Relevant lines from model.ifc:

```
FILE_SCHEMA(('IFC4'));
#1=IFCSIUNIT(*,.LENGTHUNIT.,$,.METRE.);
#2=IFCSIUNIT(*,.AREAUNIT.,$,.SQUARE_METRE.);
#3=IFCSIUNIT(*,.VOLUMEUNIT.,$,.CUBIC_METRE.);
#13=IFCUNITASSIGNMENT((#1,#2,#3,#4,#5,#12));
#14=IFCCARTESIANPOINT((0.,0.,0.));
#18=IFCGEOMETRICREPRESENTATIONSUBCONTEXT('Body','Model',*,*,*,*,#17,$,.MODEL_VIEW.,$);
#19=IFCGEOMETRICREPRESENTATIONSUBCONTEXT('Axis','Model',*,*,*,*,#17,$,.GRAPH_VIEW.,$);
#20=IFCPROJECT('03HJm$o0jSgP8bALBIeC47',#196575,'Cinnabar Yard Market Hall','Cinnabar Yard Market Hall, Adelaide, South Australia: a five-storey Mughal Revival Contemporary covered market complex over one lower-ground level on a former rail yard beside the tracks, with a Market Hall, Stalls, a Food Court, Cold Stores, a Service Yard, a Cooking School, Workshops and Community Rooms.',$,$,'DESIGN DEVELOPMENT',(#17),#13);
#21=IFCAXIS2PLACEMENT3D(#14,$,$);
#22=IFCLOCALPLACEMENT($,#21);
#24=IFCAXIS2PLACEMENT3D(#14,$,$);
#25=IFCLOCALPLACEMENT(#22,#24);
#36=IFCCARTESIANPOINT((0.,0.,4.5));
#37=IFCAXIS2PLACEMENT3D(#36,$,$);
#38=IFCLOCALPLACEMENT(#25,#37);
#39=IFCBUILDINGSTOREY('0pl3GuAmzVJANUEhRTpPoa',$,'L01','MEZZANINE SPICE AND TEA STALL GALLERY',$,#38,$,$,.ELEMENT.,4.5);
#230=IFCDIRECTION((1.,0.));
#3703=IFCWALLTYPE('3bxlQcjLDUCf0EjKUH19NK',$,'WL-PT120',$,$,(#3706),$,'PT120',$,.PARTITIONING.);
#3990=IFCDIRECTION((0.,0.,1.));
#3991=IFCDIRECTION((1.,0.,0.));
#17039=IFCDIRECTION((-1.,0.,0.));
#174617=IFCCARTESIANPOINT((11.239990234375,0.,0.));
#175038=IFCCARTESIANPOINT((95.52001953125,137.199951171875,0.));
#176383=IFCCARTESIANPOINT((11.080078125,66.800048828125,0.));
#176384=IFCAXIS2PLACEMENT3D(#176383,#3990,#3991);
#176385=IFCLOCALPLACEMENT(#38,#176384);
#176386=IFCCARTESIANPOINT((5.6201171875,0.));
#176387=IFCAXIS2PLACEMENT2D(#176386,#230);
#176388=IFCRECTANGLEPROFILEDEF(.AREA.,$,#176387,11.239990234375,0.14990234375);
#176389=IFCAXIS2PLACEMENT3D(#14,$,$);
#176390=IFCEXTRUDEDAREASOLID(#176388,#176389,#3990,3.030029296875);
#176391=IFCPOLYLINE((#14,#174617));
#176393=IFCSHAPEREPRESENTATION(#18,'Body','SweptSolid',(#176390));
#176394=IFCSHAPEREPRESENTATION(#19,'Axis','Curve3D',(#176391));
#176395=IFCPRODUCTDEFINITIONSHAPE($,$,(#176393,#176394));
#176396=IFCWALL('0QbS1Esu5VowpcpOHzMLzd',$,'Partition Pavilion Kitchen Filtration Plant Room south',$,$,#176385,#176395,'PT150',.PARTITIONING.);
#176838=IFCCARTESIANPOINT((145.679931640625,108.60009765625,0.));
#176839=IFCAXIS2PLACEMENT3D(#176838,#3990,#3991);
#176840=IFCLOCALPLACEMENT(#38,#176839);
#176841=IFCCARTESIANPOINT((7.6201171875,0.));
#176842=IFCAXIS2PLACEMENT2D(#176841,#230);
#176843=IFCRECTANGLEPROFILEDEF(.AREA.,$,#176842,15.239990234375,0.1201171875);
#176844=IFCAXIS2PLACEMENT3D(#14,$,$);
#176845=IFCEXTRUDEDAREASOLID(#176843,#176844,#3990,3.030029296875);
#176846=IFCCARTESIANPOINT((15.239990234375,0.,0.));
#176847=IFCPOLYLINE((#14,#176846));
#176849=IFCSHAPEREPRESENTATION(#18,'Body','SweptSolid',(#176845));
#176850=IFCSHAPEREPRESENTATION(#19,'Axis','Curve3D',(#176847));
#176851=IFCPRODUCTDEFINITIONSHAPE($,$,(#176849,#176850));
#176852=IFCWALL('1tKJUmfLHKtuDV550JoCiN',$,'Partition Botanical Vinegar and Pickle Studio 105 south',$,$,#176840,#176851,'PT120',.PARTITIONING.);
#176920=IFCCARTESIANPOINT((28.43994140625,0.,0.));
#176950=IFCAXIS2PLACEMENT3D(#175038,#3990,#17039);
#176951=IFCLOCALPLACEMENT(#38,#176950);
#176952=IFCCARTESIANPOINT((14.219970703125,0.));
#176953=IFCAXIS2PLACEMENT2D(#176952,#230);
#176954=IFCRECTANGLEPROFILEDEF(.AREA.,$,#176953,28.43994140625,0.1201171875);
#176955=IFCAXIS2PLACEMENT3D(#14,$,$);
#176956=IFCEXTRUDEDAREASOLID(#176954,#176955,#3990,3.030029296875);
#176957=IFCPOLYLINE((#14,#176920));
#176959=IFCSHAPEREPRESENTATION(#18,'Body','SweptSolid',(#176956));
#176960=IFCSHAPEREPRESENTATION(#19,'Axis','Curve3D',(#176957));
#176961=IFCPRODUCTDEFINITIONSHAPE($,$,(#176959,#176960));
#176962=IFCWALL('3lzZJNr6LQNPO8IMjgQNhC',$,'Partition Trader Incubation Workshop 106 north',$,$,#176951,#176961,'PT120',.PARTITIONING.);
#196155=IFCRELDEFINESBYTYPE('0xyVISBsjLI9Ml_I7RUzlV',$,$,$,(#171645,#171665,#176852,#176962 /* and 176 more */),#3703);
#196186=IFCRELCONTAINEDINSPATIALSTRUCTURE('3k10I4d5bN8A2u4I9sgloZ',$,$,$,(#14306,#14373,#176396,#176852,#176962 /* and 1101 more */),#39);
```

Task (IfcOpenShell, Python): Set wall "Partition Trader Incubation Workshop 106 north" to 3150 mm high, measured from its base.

```python
import ifcopenshell
import ifcopenshell.geom
import ifcopenshell.util.representation
import ifcopenshell.util.shape
import ifcopenshell.util.unit

model = ifcopenshell.open("model.ifc")
unit_scale = ifcopenshell.util.unit.calculate_unit_scale(model)
settings = ifcopenshell.geom.settings()


def volume(element):
    """Net volume in cubic metres, openings subtracted."""
    shape = ifcopenshell.geom.create_shape(settings, element)
    return ifcopenshell.util.shape.get_volume(shape.geometry)


wall = model.by_id(176962)
before = volume(wall)

body = ifcopenshell.util.representation.get_representation(wall, "Model", "Body")
solid = body.Items[0]
old_height = solid.Depth
solid.Depth = 3.15 / unit_scale
after = volume(wall)

print(f"height {old_height:g} -> {solid.Depth:g}, volume {before:.3f} -> {after:.3f} m3")

model.write("model_v2.ifc")
```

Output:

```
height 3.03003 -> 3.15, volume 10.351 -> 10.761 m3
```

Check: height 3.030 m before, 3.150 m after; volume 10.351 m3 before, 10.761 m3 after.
